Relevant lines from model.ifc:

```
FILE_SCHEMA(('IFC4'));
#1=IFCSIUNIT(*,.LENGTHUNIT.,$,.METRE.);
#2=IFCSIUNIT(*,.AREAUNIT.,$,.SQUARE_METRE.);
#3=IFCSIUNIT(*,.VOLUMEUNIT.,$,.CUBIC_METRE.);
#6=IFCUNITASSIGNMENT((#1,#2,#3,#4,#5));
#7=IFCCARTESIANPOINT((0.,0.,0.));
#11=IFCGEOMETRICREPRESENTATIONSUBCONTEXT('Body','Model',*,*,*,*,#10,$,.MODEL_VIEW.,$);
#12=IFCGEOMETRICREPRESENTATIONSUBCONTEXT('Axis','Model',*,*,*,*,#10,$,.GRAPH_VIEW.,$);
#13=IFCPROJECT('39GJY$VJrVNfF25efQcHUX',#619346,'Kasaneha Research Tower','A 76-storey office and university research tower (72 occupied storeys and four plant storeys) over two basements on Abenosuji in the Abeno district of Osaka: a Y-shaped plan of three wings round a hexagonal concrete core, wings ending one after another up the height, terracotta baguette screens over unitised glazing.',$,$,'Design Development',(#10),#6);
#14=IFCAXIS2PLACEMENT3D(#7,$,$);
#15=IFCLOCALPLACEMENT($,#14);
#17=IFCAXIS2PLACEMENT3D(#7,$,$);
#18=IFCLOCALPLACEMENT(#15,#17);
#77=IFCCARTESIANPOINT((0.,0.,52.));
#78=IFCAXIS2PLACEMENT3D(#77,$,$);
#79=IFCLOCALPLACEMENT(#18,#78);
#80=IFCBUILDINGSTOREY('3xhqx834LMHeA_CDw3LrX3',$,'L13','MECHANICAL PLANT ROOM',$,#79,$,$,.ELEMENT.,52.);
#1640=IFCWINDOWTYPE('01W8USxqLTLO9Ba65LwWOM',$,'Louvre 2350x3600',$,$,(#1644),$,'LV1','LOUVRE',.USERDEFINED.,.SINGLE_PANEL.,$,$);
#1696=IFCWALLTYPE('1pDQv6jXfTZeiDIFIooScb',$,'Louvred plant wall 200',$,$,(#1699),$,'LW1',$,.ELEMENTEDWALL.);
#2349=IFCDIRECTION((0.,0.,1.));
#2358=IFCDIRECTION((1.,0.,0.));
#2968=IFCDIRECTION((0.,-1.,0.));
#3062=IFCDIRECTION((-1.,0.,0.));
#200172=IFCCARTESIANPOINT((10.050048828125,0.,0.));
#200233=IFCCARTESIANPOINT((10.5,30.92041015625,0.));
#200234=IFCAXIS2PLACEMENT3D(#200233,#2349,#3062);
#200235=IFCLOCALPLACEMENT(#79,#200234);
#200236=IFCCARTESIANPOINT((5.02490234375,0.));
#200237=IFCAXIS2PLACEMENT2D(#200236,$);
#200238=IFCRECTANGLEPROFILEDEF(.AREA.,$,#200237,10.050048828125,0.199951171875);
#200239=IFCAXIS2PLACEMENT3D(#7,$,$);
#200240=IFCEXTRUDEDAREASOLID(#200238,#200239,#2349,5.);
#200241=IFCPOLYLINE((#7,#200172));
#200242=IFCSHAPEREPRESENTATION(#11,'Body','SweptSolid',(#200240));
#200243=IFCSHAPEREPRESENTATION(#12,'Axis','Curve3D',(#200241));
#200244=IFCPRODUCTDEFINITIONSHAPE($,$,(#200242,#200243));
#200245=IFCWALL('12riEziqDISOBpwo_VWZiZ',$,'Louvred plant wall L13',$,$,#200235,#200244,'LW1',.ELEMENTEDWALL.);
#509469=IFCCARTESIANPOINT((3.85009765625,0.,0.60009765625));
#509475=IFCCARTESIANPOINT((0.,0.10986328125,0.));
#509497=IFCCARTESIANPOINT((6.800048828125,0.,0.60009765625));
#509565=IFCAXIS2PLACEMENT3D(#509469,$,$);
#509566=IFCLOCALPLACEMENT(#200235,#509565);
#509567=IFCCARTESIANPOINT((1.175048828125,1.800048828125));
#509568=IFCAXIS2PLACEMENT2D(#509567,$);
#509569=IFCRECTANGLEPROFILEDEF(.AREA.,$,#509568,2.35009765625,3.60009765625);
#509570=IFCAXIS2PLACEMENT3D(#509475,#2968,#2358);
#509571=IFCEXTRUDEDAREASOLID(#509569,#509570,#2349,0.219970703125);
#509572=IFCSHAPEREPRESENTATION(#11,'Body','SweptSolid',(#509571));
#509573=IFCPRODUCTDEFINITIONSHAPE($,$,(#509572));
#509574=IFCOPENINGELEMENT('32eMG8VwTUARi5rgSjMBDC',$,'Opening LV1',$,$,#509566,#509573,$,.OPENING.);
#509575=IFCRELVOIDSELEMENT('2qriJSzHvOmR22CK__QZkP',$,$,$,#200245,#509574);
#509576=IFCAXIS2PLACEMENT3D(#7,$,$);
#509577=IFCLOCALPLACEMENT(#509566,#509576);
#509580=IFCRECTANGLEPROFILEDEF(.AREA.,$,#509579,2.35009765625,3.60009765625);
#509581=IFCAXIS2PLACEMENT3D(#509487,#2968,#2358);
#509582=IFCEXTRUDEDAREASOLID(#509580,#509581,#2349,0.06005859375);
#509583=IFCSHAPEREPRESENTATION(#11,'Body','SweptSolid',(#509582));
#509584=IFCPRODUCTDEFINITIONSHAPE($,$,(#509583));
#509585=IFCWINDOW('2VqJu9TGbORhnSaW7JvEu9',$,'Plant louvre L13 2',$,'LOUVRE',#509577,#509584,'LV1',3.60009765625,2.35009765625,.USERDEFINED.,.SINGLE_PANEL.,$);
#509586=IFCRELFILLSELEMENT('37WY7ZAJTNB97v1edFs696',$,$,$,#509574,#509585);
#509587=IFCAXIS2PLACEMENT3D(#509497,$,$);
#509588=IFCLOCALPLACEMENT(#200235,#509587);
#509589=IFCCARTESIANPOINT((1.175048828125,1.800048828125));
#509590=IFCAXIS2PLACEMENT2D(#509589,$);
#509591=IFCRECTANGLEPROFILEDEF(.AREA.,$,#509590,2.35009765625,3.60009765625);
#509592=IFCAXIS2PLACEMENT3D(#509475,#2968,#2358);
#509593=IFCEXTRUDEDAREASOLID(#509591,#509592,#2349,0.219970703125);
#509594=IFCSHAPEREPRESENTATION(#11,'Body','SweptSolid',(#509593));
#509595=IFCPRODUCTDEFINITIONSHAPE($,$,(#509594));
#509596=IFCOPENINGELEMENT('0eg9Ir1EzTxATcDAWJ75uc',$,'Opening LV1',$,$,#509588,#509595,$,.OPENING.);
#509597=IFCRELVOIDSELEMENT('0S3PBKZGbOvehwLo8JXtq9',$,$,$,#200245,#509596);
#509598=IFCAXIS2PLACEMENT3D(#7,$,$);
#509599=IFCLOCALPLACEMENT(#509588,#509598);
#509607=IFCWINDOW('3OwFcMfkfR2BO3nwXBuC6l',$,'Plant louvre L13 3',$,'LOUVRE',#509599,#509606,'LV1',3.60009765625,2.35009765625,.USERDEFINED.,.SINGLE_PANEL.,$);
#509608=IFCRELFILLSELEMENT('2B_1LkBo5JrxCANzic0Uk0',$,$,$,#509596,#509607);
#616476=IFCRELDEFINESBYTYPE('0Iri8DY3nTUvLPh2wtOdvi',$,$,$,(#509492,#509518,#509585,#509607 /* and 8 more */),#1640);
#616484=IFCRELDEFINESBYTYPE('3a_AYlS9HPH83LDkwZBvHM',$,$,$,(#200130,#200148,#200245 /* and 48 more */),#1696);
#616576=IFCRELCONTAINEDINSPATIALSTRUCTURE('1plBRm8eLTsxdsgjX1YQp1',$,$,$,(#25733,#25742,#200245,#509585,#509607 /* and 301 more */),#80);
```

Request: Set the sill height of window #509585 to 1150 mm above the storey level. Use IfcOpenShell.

```python
import numpy as np
import ifcopenshell
import ifcopenshell.api.geometry
import ifcopenshell.geom
import ifcopenshell.util.element
import ifcopenshell.util.placement
import ifcopenshell.util.shape
import ifcopenshell.util.unit

model = ifcopenshell.open("model.ifc")
unit_scale = ifcopenshell.util.unit.calculate_unit_scale(model)

window = model.by_guid("2VqJu9TGbORhnSaW7JvEu9")
opening = window.FillsVoids[0].RelatingOpeningElement
storey = ifcopenshell.util.element.get_container(window, ifc_class="IfcBuildingStorey")
level = ifcopenshell.util.placement.get_local_placement(storey.ObjectPlacement)[2, 3]

# The opening's origin need not be at the sill, so measure its lowest point.
shape = ifcopenshell.geom.create_shape(ifcopenshell.geom.settings(), opening)
bottom = ifcopenshell.util.shape.get_shape_bottom_elevation(shape, shape.geometry) / unit_scale
dz = level + 1.15 / unit_scale - bottom

shift = np.array([0.0, 0.0, dz])
# The window is placed relative to its opening, so it follows when the opening moves.
matrix = ifcopenshell.util.placement.get_local_placement(opening.ObjectPlacement)
matrix[:3, 3] += shift
ifcopenshell.api.geometry.edit_object_placement(
    model, product=opening, matrix=matrix, is_si=False, should_transform_children=True
)

print(f"moved by {dz * unit_scale:+.3f} m")

model.write("model_v2.ifc")
```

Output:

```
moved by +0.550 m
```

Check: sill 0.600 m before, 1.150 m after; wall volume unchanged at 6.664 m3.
